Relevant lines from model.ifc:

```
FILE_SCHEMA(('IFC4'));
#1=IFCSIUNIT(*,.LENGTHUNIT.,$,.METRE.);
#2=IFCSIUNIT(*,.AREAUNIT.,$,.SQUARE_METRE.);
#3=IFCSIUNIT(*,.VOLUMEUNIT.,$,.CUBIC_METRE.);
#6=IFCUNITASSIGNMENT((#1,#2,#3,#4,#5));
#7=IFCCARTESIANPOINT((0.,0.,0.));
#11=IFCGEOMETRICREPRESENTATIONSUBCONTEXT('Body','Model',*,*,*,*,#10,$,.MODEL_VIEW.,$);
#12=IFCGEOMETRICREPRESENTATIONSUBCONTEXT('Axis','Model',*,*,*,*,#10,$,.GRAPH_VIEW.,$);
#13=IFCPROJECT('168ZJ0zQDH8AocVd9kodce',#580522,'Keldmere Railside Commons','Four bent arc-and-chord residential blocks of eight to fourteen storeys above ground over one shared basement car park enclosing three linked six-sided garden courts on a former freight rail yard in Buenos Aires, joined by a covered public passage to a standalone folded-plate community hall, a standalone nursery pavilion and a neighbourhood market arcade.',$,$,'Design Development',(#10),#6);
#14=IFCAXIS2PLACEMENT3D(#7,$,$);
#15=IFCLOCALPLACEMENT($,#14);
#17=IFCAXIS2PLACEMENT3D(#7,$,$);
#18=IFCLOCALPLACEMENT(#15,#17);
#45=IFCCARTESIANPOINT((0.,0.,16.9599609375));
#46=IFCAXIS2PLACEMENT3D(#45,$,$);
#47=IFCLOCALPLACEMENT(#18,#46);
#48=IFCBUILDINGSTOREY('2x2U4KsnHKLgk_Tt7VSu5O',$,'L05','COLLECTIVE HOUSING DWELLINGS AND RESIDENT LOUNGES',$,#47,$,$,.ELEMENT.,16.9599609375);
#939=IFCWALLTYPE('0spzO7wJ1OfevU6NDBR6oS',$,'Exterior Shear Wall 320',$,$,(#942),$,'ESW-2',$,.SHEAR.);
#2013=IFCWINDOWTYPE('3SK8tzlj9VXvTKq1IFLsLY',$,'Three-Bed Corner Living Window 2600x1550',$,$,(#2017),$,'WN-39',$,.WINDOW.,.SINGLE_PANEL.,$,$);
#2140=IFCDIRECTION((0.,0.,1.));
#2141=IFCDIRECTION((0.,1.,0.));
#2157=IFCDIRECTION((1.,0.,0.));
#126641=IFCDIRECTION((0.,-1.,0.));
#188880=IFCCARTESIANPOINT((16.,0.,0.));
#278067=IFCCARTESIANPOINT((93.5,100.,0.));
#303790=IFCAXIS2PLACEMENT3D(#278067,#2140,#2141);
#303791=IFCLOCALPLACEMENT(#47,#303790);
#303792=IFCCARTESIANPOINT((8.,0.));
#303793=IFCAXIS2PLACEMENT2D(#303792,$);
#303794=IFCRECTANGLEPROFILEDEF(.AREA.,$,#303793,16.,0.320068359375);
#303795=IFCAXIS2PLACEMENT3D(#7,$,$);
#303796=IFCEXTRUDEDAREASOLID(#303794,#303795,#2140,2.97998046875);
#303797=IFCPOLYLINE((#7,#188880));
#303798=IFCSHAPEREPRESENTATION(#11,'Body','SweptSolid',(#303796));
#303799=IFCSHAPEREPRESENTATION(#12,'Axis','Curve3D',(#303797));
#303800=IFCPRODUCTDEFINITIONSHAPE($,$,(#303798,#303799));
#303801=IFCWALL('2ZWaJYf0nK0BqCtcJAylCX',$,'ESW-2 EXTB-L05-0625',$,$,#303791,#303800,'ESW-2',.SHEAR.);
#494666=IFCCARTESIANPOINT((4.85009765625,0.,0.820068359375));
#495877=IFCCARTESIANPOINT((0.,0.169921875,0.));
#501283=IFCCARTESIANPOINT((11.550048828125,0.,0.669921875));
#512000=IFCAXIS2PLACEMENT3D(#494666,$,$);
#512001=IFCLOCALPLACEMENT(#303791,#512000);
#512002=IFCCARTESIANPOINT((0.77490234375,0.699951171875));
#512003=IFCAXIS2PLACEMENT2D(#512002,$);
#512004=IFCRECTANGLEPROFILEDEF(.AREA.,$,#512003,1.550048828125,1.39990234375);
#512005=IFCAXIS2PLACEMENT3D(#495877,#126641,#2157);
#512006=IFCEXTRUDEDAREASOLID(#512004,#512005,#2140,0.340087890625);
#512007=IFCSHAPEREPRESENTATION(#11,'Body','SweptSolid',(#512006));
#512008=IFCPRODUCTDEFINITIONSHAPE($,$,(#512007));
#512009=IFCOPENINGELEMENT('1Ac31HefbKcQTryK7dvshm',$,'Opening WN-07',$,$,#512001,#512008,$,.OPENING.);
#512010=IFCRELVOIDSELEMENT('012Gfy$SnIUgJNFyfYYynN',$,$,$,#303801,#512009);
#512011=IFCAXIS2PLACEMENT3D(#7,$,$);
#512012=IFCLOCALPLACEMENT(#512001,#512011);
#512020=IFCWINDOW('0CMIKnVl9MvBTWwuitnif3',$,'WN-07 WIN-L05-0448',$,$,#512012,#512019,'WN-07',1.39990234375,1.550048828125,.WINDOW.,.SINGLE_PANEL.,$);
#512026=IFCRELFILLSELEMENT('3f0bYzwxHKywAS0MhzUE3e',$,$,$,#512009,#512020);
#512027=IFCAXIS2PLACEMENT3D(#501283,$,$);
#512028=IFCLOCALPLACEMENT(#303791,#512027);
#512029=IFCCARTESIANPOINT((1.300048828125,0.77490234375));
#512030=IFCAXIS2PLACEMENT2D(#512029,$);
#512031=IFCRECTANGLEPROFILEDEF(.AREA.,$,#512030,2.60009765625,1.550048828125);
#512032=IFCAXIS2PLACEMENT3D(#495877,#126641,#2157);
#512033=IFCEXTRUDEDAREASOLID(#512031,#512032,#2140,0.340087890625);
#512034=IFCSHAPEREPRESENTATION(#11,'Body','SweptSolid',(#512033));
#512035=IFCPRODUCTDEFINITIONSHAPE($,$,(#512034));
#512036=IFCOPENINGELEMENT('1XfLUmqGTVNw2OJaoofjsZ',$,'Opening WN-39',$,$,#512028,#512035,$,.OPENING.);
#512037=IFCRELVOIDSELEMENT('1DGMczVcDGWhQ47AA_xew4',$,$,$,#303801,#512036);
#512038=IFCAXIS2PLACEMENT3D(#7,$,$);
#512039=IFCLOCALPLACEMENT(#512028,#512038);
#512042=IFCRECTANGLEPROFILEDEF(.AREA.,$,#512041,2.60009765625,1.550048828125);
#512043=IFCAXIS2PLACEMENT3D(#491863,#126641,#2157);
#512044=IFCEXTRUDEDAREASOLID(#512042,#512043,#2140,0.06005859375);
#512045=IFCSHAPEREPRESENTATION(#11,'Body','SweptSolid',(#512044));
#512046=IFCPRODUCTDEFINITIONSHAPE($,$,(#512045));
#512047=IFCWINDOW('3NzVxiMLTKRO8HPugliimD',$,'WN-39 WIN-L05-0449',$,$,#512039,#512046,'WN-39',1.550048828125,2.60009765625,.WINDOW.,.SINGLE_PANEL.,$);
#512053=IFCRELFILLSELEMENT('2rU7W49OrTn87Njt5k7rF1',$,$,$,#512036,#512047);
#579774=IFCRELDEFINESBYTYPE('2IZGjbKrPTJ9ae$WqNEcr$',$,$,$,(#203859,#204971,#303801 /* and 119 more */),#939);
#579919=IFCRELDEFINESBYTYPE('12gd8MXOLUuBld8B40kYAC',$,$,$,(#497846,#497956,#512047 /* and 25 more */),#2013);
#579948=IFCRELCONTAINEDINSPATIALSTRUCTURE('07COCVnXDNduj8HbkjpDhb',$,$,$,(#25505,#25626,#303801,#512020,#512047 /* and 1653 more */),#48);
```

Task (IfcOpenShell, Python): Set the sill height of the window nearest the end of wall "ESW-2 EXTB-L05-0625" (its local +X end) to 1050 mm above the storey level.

```python
import numpy as np
import ifcopenshell
import ifcopenshell.api.geometry
import ifcopenshell.geom
import ifcopenshell.util.element
import ifcopenshell.util.placement
import ifcopenshell.util.shape
import ifcopenshell.util.unit

model = ifcopenshell.open("model.ifc")
unit_scale = ifcopenshell.util.unit.calculate_unit_scale(model)

window = model.by_id(512047)
opening = window.FillsVoids[0].RelatingOpeningElement
storey = ifcopenshell.util.element.get_container(window, ifc_class="IfcBuildingStorey")
level = ifcopenshell.util.placement.get_local_placement(storey.ObjectPlacement)[2, 3]

# The opening's origin need not be at the sill, so measure its lowest point.
shape = ifcopenshell.geom.create_shape(ifcopenshell.geom.settings(), opening)
bottom = ifcopenshell.util.shape.get_shape_bottom_elevation(shape, shape.geometry) / unit_scale
dz = level + 1.05 - bottom

shift = np.array([0.0, 0.0, dz])
# The window is placed relative to its opening, so it follows when the opening moves.
matrix = ifcopenshell.util.placement.get_local_placement(opening.ObjectPlacement)
matrix[:3, 3] += shift
ifcopenshell.api.geometry.edit_object_placement(
    model, product=opening, matrix=matrix, is_si=False, should_transform_children=True
)

print(f"moved by {dz * unit_scale:+.3f} m")

model.write("model_rev.ifc")
```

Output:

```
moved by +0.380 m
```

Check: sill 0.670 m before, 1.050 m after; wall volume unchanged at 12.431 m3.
